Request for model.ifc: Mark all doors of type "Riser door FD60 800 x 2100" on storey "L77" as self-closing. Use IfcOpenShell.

First a look at what the model holds.

```python
import ifcopenshell
import ifcopenshell.util.element

model = ifcopenshell.open("model.ifc")
print(model.schema)
storey = next(s for s in model.by_type("IfcBuildingStorey") if s.Name == "L77")
doors = [e for e in ifcopenshell.util.element.get_decomposition(storey) if e.is_a("IfcDoor")]
seen = {}
for e in doors:
    element_type = ifcopenshell.util.element.get_type(e)
    key = (element_type.Name if element_type != e and element_type else None, ifcopenshell.util.element.get_pset(e, "Pset_DoorCommon", "SelfClosing"))
    seen[key] = seen.get(key, 0) + 1
for (name, value), count in sorted(seen.items(), key=str):
    print(count, "x", name, "|", value)
```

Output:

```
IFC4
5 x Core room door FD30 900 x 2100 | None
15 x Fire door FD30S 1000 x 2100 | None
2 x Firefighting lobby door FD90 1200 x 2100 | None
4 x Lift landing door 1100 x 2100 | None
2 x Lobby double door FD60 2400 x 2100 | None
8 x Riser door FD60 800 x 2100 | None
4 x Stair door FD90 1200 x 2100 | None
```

```python
import ifcopenshell
import ifcopenshell.api.pset
import ifcopenshell.util.element

model = ifcopenshell.open("model.ifc")

storey = next(s for s in model.by_type("IfcBuildingStorey") if s.Name == "L77")
doors = [e for e in ifcopenshell.util.element.get_decomposition(storey) if e.is_a("IfcDoor")]

count = 0
for e in doors:
    element_type = ifcopenshell.util.element.get_type(e)
    if element_type in (None, e) or element_type.Name != "Riser door FD60 800 x 2100":
        continue
    # add_pset returns the element's existing set when there is one.
    pset = ifcopenshell.api.pset.add_pset(model, product=e, name="Pset_DoorCommon")
    ifcopenshell.api.pset.edit_pset(model, pset=pset, properties={"SelfClosing": True})
    count += 1

print(count, "doors updated")

model.write("model-out.ifc")
```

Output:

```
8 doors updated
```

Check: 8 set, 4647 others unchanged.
